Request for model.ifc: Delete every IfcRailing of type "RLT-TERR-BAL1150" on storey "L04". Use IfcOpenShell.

First a look at what the model holds.

```python
import ifcopenshell
import ifcopenshell.util.element

model = ifcopenshell.open("model.ifc")
print(model.schema)
storey = next(s for s in model.by_type("IfcBuildingStorey") if s.Name == "L04")
railings = [e for e in ifcopenshell.util.element.get_decomposition(storey) if e.is_a("IfcRailing")]
seen = {}
for e in railings:
    element_type = ifcopenshell.util.element.get_type(e)
    name = element_type.Name if element_type not in (None, e) else None
    seen[name] = seen.get(name, 0) + 1
for name, count in sorted(seen.items(), key=str):
    print(count, "x", name)
```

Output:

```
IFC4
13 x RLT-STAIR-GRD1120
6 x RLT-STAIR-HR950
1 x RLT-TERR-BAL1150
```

```python
import ifcopenshell
import ifcopenshell.api.root
import ifcopenshell.util.element

model = ifcopenshell.open("model.ifc")

storey = next(s for s in model.by_type("IfcBuildingStorey") if s.Name == "L04")
railings = [e for e in ifcopenshell.util.element.get_decomposition(storey) if e.is_a("IfcRailing")]
targets = [e for e in railings if (t := ifcopenshell.util.element.get_type(e)) not in (None, e) and t.Name == "RLT-TERR-BAL1150"]

for e in targets:
    ifcopenshell.api.root.remove_product(model, product=e)
print(len(targets), "removed")

model.write("model-out.ifc")
```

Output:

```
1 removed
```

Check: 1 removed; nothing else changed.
